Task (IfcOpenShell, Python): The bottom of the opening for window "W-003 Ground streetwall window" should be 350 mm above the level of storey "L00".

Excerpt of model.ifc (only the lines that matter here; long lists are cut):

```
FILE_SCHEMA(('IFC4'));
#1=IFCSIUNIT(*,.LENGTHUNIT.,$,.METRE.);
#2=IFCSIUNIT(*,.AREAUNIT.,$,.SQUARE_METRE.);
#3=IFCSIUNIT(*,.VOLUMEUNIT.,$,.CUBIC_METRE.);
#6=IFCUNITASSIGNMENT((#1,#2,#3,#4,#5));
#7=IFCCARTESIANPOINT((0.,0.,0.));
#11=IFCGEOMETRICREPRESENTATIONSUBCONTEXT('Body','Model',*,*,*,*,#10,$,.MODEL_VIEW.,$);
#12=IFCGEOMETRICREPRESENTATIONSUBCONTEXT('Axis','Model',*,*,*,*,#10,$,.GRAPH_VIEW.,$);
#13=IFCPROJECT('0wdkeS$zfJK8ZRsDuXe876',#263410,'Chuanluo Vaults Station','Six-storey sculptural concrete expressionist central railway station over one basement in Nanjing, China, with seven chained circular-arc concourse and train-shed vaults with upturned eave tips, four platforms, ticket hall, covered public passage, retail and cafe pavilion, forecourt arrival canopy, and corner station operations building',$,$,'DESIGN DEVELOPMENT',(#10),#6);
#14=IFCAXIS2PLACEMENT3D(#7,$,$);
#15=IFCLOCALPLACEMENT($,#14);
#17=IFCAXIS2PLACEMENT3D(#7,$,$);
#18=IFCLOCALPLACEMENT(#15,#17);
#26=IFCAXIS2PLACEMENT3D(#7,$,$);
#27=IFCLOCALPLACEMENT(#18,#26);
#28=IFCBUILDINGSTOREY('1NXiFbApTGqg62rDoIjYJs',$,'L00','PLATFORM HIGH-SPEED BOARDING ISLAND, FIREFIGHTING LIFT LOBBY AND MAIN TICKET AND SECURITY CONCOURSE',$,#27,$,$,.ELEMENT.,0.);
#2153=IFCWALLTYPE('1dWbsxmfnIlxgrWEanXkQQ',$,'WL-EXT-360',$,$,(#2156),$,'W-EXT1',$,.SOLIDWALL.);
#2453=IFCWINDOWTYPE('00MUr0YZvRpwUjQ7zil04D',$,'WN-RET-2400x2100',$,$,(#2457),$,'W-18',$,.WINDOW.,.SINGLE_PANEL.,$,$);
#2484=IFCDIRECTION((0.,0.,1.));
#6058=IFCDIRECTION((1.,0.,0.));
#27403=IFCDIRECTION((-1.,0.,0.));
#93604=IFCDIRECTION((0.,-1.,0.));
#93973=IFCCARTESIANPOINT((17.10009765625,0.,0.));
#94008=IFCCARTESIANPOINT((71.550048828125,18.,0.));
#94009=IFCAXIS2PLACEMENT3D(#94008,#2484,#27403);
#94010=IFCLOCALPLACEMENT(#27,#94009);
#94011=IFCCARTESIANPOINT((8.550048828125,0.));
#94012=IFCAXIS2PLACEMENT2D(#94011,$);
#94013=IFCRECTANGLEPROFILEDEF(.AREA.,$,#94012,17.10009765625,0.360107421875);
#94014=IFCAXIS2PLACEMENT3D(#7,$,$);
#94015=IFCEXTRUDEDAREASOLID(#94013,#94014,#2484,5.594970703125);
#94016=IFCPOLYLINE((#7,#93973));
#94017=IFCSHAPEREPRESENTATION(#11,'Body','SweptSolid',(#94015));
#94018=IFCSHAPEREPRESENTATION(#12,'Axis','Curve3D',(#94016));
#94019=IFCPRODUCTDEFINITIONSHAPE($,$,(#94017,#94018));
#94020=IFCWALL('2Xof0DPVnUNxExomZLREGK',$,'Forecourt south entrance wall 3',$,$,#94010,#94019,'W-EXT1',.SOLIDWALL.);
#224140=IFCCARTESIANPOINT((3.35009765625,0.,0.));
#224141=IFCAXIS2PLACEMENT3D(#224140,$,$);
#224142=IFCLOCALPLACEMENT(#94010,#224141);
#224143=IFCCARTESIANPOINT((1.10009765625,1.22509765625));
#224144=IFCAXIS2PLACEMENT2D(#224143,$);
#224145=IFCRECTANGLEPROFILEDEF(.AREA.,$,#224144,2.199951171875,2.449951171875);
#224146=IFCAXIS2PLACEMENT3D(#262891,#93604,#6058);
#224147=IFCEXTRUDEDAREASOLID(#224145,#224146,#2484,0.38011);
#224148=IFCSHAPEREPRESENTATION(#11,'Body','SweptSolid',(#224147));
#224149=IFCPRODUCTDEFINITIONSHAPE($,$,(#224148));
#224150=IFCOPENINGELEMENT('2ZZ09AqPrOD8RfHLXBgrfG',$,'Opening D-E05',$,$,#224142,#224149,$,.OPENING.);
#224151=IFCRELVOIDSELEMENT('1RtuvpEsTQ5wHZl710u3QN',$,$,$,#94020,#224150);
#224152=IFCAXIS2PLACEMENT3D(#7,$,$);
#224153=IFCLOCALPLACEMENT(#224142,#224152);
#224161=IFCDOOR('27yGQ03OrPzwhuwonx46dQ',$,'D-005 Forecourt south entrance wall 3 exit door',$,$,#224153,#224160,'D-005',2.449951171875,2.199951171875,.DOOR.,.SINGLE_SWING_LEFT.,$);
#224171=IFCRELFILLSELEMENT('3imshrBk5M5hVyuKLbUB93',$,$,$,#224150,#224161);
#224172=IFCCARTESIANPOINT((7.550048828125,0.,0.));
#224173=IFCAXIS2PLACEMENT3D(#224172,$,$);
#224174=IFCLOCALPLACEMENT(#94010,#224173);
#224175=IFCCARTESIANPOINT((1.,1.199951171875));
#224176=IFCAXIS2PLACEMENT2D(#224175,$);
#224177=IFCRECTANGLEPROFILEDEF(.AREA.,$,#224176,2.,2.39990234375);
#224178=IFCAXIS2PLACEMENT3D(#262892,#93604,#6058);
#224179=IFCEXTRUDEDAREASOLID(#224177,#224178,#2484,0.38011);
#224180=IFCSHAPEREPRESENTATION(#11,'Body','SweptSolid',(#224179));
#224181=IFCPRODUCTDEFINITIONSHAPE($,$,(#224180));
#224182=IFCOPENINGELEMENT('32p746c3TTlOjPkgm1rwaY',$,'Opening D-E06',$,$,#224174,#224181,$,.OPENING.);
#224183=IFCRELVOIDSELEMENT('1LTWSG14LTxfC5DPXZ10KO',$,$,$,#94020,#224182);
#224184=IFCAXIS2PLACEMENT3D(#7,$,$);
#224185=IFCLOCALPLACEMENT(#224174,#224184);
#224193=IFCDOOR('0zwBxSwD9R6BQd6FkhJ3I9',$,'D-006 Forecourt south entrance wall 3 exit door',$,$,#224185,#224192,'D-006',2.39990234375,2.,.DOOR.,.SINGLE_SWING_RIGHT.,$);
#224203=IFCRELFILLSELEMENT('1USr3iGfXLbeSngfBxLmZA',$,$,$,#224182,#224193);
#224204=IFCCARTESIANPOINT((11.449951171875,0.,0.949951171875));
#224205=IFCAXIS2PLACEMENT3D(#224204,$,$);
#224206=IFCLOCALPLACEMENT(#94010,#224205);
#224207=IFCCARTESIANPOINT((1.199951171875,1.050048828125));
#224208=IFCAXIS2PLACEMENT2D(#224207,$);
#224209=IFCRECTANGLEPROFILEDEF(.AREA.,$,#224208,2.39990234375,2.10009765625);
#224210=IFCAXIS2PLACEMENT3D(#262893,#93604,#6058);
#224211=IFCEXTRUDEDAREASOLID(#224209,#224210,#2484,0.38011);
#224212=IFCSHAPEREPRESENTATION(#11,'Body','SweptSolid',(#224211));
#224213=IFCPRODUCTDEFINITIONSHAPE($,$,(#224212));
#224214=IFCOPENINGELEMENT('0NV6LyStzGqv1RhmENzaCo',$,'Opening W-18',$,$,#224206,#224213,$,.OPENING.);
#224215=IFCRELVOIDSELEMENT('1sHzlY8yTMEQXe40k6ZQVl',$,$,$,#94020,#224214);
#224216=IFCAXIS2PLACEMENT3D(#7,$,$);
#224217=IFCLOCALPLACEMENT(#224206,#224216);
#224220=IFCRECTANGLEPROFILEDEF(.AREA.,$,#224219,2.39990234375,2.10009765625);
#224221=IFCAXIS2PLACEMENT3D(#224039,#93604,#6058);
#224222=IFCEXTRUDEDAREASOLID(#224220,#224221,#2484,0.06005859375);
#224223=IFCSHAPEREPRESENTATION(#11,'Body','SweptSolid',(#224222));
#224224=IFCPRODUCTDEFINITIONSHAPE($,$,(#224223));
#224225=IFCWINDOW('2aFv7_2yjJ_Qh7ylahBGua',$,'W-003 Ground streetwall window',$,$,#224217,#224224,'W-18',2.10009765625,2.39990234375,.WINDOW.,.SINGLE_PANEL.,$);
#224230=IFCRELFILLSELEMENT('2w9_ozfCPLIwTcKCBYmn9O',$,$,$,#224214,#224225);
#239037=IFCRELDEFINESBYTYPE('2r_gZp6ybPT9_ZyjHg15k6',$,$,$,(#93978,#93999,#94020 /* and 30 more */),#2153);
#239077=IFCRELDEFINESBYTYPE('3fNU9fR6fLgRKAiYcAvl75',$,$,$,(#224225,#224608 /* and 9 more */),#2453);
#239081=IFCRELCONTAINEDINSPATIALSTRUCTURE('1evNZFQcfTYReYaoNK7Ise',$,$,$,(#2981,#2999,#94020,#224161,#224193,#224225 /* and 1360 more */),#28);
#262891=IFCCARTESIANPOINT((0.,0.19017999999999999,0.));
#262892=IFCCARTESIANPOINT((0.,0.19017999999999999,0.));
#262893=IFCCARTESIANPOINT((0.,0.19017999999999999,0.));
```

```python
import numpy as np
import ifcopenshell
import ifcopenshell.api.geometry
import ifcopenshell.geom
import ifcopenshell.util.element
import ifcopenshell.util.placement
import ifcopenshell.util.shape
import ifcopenshell.util.unit

model = ifcopenshell.open("model.ifc")
unit_scale = ifcopenshell.util.unit.calculate_unit_scale(model)

window = model.by_guid("2aFv7_2yjJ_Qh7ylahBGua")
opening = window.FillsVoids[0].RelatingOpeningElement
storey = ifcopenshell.util.element.get_container(window, ifc_class="IfcBuildingStorey")
level = ifcopenshell.util.placement.get_local_placement(storey.ObjectPlacement)[2, 3]

# The opening's origin need not be at the sill, so measure its lowest point.
shape = ifcopenshell.geom.create_shape(ifcopenshell.geom.settings(), opening)
bottom = ifcopenshell.util.shape.get_shape_bottom_elevation(shape, shape.geometry) / unit_scale
dz = level + 0.35 / unit_scale - bottom

shift = np.array([0.0, 0.0, dz])
# The window is placed relative to its opening, so it follows when the opening moves.
matrix = ifcopenshell.util.placement.get_local_placement(opening.ObjectPlacement)
matrix[:3, 3] += shift
ifcopenshell.api.geometry.edit_object_placement(
    model, product=opening, matrix=matrix, is_si=False, should_transform_children=True
)

print(f"moved by {dz * unit_scale:+.3f} m")

model.write("model_rev.ifc")
```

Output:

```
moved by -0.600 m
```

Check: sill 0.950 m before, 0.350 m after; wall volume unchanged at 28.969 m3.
